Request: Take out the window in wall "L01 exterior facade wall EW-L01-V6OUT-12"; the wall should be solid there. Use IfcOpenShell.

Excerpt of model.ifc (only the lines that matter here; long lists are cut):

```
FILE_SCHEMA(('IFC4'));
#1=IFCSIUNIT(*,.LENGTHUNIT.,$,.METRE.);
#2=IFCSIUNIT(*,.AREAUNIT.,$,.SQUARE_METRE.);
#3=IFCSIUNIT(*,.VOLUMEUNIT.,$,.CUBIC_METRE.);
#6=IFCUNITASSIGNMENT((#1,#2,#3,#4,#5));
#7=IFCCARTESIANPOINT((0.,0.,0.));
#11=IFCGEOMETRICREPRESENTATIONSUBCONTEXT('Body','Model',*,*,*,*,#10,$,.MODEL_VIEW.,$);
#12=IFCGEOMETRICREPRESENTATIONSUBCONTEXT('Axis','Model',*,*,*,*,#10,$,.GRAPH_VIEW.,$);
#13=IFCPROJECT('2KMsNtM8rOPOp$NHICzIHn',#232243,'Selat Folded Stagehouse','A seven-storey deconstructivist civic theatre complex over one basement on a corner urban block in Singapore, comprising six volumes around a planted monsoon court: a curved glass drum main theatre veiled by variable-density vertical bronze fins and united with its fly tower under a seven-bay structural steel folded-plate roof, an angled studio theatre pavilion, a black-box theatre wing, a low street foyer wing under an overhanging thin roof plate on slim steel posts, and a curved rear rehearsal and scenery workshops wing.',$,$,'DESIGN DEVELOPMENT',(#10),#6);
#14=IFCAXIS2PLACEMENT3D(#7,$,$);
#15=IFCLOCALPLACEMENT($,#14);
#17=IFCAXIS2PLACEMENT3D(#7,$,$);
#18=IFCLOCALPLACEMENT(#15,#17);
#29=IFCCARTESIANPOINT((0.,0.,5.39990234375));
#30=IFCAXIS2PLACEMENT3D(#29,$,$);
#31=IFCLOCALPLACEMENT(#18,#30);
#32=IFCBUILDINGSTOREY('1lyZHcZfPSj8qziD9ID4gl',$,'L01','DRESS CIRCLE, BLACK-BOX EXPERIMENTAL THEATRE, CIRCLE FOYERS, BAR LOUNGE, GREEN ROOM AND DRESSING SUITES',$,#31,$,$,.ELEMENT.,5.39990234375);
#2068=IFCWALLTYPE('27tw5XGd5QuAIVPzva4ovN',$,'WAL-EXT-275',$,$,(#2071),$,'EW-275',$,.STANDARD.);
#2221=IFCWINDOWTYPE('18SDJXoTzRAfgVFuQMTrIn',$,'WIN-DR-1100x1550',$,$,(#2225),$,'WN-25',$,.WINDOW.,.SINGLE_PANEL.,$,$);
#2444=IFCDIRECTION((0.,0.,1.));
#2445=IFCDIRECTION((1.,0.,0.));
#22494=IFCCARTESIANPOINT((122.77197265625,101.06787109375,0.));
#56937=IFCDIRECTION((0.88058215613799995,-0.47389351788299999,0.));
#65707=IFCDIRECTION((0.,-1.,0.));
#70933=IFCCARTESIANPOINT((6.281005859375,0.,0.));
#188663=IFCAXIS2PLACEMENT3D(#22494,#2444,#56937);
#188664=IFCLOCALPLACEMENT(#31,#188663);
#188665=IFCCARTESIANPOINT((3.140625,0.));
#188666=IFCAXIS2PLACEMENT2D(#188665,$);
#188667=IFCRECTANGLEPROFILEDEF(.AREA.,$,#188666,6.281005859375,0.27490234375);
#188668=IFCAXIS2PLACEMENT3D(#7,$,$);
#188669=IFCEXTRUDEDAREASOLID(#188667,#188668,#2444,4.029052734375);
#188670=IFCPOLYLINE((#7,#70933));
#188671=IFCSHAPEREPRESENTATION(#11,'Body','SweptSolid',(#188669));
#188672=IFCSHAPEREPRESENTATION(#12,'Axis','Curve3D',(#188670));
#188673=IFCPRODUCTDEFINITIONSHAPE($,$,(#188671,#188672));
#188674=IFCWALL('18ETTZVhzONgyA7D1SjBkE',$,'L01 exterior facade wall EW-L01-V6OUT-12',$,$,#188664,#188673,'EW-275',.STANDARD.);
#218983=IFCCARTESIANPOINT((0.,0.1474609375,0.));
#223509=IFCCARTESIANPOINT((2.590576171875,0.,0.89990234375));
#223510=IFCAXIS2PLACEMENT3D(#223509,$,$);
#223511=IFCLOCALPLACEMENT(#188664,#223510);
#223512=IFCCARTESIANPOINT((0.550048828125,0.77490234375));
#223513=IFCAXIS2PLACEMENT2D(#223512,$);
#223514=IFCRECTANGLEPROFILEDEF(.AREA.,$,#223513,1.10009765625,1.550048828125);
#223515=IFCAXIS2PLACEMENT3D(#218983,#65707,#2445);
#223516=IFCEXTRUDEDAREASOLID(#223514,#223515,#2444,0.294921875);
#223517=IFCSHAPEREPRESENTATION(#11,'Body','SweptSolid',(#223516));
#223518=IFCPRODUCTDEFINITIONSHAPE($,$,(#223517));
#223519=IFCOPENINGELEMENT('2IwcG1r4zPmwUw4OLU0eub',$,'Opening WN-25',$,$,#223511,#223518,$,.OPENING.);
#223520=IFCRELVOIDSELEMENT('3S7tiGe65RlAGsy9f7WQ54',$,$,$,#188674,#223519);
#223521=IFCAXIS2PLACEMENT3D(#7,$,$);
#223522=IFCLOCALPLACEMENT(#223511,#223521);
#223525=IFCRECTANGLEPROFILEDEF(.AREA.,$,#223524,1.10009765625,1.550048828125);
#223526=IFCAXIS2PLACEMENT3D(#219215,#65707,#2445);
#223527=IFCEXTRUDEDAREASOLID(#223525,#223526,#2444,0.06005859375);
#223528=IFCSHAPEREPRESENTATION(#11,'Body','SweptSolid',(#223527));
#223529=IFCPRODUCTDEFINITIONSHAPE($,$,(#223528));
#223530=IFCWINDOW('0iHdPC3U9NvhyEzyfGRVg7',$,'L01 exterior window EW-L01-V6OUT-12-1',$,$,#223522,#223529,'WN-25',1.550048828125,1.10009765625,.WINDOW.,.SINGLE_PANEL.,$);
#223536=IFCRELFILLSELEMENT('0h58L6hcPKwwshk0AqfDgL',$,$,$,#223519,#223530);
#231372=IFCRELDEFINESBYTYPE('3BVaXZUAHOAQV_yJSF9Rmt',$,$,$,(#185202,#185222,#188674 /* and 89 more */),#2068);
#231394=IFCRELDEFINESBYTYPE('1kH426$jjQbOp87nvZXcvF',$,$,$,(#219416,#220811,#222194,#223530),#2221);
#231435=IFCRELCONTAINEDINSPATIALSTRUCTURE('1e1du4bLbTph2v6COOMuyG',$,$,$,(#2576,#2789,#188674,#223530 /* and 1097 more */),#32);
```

```python
import ifcopenshell
import ifcopenshell.api.feature
import ifcopenshell.api.root
import ifcopenshell.geom
import ifcopenshell.util.shape

model = ifcopenshell.open("model.ifc")
settings = ifcopenshell.geom.settings()


def volume(element):
    """Net volume in cubic metres, openings subtracted."""
    shape = ifcopenshell.geom.create_shape(settings, element)
    return ifcopenshell.util.shape.get_volume(shape.geometry)


window = model.by_guid("0iHdPC3U9NvhyEzyfGRVg7")
opening = window.FillsVoids[0].RelatingOpeningElement
wall = opening.VoidsElements[0].RelatingBuildingElement
before = volume(wall)

ifcopenshell.api.root.remove_product(model, product=window)
ifcopenshell.api.feature.remove_feature(model, feature=opening)

after = volume(wall)

print(f"wall volume {before:.3f} -> {after:.3f} m3")

model.write("model-out.ifc")
```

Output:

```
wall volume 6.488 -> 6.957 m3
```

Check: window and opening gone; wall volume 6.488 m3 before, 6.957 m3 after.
